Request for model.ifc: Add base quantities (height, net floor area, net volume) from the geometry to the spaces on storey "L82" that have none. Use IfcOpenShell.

First a look at what the model holds.

```python
import ifcopenshell
import ifcopenshell.util.element
import ifcopenshell.util.unit

model = ifcopenshell.open("model.ifc")
print(model.schema)
for unit_type in ("LENGTHUNIT", "AREAUNIT", "VOLUMEUNIT"):
    print(unit_type, ifcopenshell.util.unit.calculate_unit_scale(model, unit_type))
storey = next(s for s in model.by_type("IfcBuildingStorey") if s.Name == "L82")
spaces = [e for e in ifcopenshell.util.element.get_decomposition(storey) if e.is_a("IfcSpace")]
for e in sorted(spaces, key=lambda e: e.id()):
    print(e.id(), e.is_a(), e.Name, list(ifcopenshell.util.element.get_psets(e, qtos_only=True)), sep=" | ")
```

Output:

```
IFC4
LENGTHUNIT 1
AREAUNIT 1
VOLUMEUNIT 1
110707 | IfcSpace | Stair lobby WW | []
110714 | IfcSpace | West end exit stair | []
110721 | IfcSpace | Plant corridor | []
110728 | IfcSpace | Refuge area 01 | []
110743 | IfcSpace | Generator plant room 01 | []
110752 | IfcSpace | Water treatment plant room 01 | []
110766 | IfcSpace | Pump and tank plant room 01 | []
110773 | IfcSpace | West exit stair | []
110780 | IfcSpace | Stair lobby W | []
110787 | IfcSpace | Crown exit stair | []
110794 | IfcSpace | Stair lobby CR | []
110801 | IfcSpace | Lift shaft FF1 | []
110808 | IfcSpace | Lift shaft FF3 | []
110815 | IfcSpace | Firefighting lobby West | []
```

```python
import ifcopenshell
import ifcopenshell.api.pset
import ifcopenshell.geom
import ifcopenshell.util.element
import ifcopenshell.util.shape
import ifcopenshell.util.unit

model = ifcopenshell.open("model.ifc")
unit_scale = ifcopenshell.util.unit.calculate_unit_scale(model)
area_scale = ifcopenshell.util.unit.calculate_unit_scale(model, "AREAUNIT")
volume_scale = ifcopenshell.util.unit.calculate_unit_scale(model, "VOLUMEUNIT")
settings = ifcopenshell.geom.settings()

storey = next(s for s in model.by_type("IfcBuildingStorey") if s.Name == "L82")
spaces = [e for e in ifcopenshell.util.element.get_decomposition(storey) if e.is_a("IfcSpace")]

for e in sorted(spaces, key=lambda e: e.id()):
    if ifcopenshell.util.element.get_psets(e, qtos_only=True, should_inherit=False):
        continue
    # Geometry comes back in metres, in the element's own axes.
    shape = ifcopenshell.geom.create_shape(settings, e)
    values = {
        "Height": ifcopenshell.util.shape.get_z(shape.geometry) / unit_scale,
        "NetFloorArea": ifcopenshell.util.shape.get_footprint_area(shape.geometry) / area_scale,
        "NetVolume": ifcopenshell.util.shape.get_volume(shape.geometry) / volume_scale,
    }
    qto = ifcopenshell.api.pset.add_qto(model, product=e, name="Qto_SpaceBaseQuantities")
    ifcopenshell.api.pset.edit_qto(model, qto=qto, properties=values)
    print(e.id(), {k: round(v, 3) for k, v in values.items()})

model.write("model_updated.ifc")
```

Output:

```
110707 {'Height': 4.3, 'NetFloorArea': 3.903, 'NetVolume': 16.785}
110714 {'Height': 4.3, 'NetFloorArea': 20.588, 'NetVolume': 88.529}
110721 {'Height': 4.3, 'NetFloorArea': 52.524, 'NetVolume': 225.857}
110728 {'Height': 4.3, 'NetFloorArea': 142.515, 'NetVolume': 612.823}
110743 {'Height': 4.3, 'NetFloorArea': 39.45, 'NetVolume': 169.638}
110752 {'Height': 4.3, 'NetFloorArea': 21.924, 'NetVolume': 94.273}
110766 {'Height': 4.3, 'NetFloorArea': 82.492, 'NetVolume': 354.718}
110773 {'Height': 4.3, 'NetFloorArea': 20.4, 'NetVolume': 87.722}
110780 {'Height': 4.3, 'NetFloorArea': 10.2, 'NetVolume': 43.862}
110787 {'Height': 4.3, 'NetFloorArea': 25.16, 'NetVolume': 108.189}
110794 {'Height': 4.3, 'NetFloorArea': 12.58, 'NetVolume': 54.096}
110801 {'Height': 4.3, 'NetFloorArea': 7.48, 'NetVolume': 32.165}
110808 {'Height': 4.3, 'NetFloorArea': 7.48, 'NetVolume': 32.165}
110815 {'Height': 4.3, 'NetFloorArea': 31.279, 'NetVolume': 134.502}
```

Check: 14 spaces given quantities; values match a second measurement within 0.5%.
